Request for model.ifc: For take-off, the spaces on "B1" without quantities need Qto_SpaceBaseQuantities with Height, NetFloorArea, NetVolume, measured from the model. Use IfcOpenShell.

First a look at what the model holds.

```python
import ifcopenshell
import ifcopenshell.util.element
import ifcopenshell.util.unit

model = ifcopenshell.open("model.ifc")
print(model.schema)
for unit_type in ("LENGTHUNIT", "AREAUNIT", "VOLUMEUNIT"):
    print(unit_type, ifcopenshell.util.unit.calculate_unit_scale(model, unit_type))
storey = next(s for s in model.by_type("IfcBuildingStorey") if s.Name == "B1")
spaces = [e for e in ifcopenshell.util.element.get_decomposition(storey) if e.is_a("IfcSpace")]
for e in sorted(spaces, key=lambda e: e.id()):
    print(e.id(), e.is_a(), e.Name, list(ifcopenshell.util.element.get_psets(e, qtos_only=True)), sep=" | ")
```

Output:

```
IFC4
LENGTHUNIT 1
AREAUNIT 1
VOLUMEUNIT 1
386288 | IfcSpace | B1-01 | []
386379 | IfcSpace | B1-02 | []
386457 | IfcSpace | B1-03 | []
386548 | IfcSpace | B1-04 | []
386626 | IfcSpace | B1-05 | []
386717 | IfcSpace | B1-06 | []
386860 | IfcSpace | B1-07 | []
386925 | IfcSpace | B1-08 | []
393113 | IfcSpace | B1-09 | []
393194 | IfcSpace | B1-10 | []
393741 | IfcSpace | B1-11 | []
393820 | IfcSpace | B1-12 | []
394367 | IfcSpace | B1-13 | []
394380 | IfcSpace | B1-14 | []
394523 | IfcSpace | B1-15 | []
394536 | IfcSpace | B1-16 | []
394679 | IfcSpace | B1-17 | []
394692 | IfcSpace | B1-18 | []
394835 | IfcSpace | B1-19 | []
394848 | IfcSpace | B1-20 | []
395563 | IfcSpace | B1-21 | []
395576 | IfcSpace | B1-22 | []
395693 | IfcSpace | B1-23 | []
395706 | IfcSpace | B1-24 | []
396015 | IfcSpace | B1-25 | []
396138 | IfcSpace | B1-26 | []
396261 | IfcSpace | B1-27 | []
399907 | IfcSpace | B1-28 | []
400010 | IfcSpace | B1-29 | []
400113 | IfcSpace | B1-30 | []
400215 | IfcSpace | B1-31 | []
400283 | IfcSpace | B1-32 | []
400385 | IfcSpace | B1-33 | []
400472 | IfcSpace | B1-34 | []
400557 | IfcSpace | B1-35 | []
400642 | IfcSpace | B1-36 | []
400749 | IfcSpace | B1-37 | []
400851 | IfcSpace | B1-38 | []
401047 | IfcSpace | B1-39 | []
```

```python
import ifcopenshell
import ifcopenshell.api.pset
import ifcopenshell.geom
import ifcopenshell.util.element
import ifcopenshell.util.shape
import ifcopenshell.util.unit

model = ifcopenshell.open("model.ifc")
unit_scale = ifcopenshell.util.unit.calculate_unit_scale(model)
area_scale = ifcopenshell.util.unit.calculate_unit_scale(model, "AREAUNIT")
volume_scale = ifcopenshell.util.unit.calculate_unit_scale(model, "VOLUMEUNIT")
settings = ifcopenshell.geom.settings()

storey = next(s for s in model.by_type("IfcBuildingStorey") if s.Name == "B1")
spaces = [e for e in ifcopenshell.util.element.get_decomposition(storey) if e.is_a("IfcSpace")]

for e in sorted(spaces, key=lambda e: e.id()):
    if ifcopenshell.util.element.get_psets(e, qtos_only=True, should_inherit=False):
        continue
    # Geometry comes back in metres, in the element's own axes.
    shape = ifcopenshell.geom.create_shape(settings, e)
    values = {
        "Height": ifcopenshell.util.shape.get_z(shape.geometry) / unit_scale,
        "NetFloorArea": ifcopenshell.util.shape.get_footprint_area(shape.geometry) / area_scale,
        "NetVolume": ifcopenshell.util.shape.get_volume(shape.geometry) / volume_scale,
    }
    qto = ifcopenshell.api.pset.add_qto(model, product=e, name="Qto_SpaceBaseQuantities")
    ifcopenshell.api.pset.edit_qto(model, qto=qto, properties=values)
    print(e.id(), {k: round(v, 3) for k, v in values.items()})

model.write("model_edited.ifc")
```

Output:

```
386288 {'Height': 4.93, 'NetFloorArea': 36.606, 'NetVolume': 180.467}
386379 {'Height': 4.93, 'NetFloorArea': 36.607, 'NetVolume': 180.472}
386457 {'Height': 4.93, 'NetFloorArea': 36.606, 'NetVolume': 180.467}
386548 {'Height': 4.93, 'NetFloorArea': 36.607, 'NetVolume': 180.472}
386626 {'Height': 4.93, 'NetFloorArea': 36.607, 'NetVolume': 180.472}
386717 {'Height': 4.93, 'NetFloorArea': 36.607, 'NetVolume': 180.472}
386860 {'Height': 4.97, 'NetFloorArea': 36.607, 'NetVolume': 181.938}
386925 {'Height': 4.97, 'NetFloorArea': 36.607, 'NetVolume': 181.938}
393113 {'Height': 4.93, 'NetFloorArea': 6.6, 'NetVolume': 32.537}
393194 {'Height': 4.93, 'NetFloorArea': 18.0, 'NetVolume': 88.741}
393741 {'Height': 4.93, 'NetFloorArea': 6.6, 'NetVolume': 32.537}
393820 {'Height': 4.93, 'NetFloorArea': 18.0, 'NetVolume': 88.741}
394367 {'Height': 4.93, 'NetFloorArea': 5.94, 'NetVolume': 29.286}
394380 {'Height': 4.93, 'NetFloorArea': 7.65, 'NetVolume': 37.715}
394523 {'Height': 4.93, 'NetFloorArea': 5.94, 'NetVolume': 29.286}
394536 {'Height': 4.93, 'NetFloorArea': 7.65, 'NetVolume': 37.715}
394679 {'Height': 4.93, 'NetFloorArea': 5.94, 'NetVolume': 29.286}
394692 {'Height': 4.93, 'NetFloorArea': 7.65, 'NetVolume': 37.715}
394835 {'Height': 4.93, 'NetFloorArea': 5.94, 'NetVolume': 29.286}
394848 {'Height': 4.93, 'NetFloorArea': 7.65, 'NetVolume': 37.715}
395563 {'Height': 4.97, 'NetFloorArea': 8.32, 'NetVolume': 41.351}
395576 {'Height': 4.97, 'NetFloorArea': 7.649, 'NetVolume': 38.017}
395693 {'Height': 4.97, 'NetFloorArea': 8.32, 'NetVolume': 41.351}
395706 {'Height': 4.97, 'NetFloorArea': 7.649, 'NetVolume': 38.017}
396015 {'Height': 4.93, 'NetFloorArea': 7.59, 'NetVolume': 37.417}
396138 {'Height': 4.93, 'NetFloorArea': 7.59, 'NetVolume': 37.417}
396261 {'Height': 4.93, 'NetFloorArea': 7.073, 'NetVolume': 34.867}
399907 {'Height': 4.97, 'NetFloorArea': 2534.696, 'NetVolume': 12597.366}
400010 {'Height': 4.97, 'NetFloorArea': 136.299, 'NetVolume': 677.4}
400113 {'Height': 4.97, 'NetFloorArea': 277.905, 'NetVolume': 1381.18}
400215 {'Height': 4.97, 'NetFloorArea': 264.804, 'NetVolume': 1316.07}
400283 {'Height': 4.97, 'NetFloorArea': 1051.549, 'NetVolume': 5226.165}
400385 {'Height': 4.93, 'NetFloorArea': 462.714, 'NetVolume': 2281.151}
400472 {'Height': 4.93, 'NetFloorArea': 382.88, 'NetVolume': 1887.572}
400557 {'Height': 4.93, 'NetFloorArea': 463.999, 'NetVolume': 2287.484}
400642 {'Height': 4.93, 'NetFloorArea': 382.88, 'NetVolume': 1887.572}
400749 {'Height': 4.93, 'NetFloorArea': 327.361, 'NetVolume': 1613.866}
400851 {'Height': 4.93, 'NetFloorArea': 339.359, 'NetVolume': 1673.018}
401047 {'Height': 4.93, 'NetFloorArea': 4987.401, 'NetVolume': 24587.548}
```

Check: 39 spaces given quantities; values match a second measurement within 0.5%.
